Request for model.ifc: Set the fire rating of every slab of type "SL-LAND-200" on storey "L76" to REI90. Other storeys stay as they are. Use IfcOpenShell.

First a look at what the model holds.

```python
import ifcopenshell
import ifcopenshell.util.element

model = ifcopenshell.open("model.ifc")
print(model.schema)
storey = next(s for s in model.by_type("IfcBuildingStorey") if s.Name == "L76")
slabs = [e for e in ifcopenshell.util.element.get_decomposition(storey) if e.is_a("IfcSlab")]
seen = {}
for e in slabs:
    element_type = ifcopenshell.util.element.get_type(e)
    key = (element_type.Name if element_type != e and element_type else None, ifcopenshell.util.element.get_pset(e, "Pset_SlabCommon", "FireRating"))
    seen[key] = seen.get(key, 0) + 1
for (name, value), count in sorted(seen.items(), key=str):
    print(count, "x", name, "|", value)
```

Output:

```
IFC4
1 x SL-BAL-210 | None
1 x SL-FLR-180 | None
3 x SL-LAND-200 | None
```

```python
import ifcopenshell
import ifcopenshell.api.pset
import ifcopenshell.util.element

model = ifcopenshell.open("model.ifc")

storey = next(s for s in model.by_type("IfcBuildingStorey") if s.Name == "L76")
slabs = [e for e in ifcopenshell.util.element.get_decomposition(storey) if e.is_a("IfcSlab")]

count = 0
for e in slabs:
    element_type = ifcopenshell.util.element.get_type(e)
    if element_type in (None, e) or element_type.Name != "SL-LAND-200":
        continue
    # add_pset returns the element's existing set when there is one.
    pset = ifcopenshell.api.pset.add_pset(model, product=e, name="Pset_SlabCommon")
    ifcopenshell.api.pset.edit_pset(model, pset=pset, properties={"FireRating": "REI90"})
    count += 1

print(count, "slabs updated")

model.write("model_edited.ifc")
```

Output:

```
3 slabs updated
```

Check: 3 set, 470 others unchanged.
